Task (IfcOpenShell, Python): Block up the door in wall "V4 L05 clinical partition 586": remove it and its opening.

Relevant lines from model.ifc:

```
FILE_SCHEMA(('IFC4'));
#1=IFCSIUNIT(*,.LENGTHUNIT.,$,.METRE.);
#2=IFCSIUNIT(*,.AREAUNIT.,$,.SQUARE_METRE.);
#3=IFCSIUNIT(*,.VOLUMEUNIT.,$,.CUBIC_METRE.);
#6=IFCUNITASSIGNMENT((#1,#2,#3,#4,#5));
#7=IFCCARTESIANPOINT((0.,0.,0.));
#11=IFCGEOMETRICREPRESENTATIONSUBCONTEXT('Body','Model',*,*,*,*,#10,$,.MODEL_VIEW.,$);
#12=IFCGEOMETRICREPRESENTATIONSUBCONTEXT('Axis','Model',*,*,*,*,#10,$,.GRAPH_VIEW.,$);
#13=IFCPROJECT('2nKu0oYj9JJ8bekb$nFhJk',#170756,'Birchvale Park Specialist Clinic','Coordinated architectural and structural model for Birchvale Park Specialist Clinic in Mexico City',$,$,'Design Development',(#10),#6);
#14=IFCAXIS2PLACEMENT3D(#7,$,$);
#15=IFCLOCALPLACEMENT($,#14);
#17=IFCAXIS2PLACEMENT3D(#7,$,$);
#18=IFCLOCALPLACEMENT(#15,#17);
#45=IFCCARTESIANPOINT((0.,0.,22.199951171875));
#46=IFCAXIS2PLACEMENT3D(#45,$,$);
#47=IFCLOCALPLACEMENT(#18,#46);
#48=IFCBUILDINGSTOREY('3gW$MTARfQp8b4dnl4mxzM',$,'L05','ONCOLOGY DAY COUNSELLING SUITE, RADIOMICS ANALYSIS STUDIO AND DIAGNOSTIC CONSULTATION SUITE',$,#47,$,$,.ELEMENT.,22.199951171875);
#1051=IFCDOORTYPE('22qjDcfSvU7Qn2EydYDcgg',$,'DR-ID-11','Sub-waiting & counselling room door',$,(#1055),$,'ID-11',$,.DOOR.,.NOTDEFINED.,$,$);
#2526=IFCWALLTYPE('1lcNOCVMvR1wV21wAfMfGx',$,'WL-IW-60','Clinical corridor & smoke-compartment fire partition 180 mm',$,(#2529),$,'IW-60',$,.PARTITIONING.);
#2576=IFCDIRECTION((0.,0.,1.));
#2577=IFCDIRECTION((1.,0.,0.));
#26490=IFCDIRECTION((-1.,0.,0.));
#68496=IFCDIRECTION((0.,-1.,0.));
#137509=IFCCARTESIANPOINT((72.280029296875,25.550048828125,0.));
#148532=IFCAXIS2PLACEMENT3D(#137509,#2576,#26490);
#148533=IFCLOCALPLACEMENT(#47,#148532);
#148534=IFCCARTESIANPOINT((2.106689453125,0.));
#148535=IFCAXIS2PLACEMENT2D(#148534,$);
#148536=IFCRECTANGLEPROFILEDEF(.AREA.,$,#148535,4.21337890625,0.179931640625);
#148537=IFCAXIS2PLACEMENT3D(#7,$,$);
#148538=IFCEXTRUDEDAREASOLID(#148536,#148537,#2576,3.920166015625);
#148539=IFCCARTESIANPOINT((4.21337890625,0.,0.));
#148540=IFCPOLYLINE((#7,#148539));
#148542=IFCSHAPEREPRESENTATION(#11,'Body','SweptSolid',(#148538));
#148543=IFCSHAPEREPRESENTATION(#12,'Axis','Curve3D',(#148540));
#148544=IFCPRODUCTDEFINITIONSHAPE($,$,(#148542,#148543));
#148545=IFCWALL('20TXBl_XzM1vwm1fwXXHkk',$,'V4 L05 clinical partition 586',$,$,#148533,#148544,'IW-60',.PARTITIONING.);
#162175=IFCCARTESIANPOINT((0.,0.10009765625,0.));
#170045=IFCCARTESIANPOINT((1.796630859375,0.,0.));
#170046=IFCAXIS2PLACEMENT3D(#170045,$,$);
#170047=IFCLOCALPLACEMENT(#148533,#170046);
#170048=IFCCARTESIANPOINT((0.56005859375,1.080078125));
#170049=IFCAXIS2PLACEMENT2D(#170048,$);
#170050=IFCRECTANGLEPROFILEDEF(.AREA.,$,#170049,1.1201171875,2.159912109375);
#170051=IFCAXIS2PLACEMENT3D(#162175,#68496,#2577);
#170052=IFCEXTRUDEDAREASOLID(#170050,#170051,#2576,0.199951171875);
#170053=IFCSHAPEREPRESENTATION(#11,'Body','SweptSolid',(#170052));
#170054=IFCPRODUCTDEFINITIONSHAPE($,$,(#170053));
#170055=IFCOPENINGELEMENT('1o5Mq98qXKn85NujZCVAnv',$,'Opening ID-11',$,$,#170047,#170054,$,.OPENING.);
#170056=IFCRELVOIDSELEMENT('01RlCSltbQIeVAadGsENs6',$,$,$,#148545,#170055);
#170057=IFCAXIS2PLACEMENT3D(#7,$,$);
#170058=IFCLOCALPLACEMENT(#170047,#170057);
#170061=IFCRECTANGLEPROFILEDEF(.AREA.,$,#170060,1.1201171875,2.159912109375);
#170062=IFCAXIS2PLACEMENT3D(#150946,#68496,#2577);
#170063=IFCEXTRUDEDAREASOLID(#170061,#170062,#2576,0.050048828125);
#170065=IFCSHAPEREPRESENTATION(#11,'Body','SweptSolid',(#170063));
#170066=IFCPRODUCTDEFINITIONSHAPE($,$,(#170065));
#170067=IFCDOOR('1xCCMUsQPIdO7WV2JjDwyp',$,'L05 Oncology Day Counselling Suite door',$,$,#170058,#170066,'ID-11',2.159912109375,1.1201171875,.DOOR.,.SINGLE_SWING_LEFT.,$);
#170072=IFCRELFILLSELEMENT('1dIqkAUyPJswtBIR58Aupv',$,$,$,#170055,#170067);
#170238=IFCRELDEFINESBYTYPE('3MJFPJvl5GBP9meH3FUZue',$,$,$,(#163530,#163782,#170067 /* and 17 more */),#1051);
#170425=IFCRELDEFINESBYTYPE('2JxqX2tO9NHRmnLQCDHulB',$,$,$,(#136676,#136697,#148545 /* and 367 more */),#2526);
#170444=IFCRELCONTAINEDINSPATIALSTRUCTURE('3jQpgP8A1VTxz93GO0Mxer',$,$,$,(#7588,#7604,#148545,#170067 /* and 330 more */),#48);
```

```python
import ifcopenshell
import ifcopenshell.api.feature
import ifcopenshell.api.root
import ifcopenshell.geom
import ifcopenshell.util.shape

model = ifcopenshell.open("model.ifc")
settings = ifcopenshell.geom.settings()


def volume(element):
    """Net volume in cubic metres, openings subtracted."""
    shape = ifcopenshell.geom.create_shape(settings, element)
    return ifcopenshell.util.shape.get_volume(shape.geometry)


door = model.by_guid("1xCCMUsQPIdO7WV2JjDwyp")
opening = door.FillsVoids[0].RelatingOpeningElement
wall = opening.VoidsElements[0].RelatingBuildingElement
before = volume(wall)

ifcopenshell.api.root.remove_product(model, product=door)
ifcopenshell.api.feature.remove_feature(model, feature=opening)

after = volume(wall)

print(f"wall volume {before:.3f} -> {after:.3f} m3")

model.write("model_v2.ifc")
```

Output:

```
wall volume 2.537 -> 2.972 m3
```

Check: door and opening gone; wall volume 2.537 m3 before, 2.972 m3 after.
